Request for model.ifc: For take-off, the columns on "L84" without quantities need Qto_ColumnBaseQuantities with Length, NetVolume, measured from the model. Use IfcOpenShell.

First a look at what the model holds.

```python
import ifcopenshell
import ifcopenshell.util.element
import ifcopenshell.util.unit

model = ifcopenshell.open("model.ifc")
print(model.schema)
for unit_type in ("LENGTHUNIT", "AREAUNIT", "VOLUMEUNIT"):
    print(unit_type, ifcopenshell.util.unit.calculate_unit_scale(model, unit_type))
storey = next(s for s in model.by_type("IfcBuildingStorey") if s.Name == "L84")
columns = [e for e in ifcopenshell.util.element.get_decomposition(storey) if e.is_a("IfcColumn")]
for e in sorted(columns, key=lambda e: e.id()):
    print(e.id(), e.is_a(), e.Name, list(ifcopenshell.util.element.get_psets(e, qtos_only=True)), sep=" | ")
```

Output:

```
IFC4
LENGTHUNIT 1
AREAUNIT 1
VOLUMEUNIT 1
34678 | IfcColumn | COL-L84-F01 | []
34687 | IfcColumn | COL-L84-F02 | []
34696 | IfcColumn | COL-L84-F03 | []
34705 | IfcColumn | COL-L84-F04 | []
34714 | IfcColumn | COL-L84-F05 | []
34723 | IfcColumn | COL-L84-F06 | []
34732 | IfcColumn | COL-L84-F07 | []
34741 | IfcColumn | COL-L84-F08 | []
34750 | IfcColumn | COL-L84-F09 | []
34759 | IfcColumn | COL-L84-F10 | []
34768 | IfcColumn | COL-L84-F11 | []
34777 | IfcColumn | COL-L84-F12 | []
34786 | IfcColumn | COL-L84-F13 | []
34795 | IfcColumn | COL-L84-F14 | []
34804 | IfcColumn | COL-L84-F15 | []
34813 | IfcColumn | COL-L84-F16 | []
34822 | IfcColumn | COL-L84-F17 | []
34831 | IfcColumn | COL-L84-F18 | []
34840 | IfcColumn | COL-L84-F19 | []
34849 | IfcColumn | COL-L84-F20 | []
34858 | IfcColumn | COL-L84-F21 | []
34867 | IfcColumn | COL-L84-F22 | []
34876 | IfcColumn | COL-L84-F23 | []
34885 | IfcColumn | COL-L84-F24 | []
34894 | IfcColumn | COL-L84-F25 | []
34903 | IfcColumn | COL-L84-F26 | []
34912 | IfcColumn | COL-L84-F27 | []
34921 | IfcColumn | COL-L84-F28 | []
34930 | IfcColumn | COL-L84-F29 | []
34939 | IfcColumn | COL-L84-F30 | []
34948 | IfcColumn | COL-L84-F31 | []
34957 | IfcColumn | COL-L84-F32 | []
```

```python
import ifcopenshell
import ifcopenshell.api.pset
import ifcopenshell.geom
import ifcopenshell.util.element
import ifcopenshell.util.shape
import ifcopenshell.util.unit

model = ifcopenshell.open("model.ifc")
unit_scale = ifcopenshell.util.unit.calculate_unit_scale(model)
volume_scale = ifcopenshell.util.unit.calculate_unit_scale(model, "VOLUMEUNIT")
settings = ifcopenshell.geom.settings()

storey = next(s for s in model.by_type("IfcBuildingStorey") if s.Name == "L84")
columns = [e for e in ifcopenshell.util.element.get_decomposition(storey) if e.is_a("IfcColumn")]

for e in sorted(columns, key=lambda e: e.id()):
    if ifcopenshell.util.element.get_psets(e, qtos_only=True, should_inherit=False):
        continue
    # Geometry comes back in metres, in the element's own axes.
    shape = ifcopenshell.geom.create_shape(settings, e)
    values = {
        "Length": ifcopenshell.util.shape.get_z(shape.geometry) / unit_scale,
        "NetVolume": ifcopenshell.util.shape.get_volume(shape.geometry) / volume_scale,
    }
    qto = ifcopenshell.api.pset.add_qto(model, product=e, name="Qto_ColumnBaseQuantities")
    ifcopenshell.api.pset.edit_qto(model, qto=qto, properties=values)
    print(e.id(), {k: round(v, 3) for k, v in values.items()})

model.write("model_v2.ifc")
```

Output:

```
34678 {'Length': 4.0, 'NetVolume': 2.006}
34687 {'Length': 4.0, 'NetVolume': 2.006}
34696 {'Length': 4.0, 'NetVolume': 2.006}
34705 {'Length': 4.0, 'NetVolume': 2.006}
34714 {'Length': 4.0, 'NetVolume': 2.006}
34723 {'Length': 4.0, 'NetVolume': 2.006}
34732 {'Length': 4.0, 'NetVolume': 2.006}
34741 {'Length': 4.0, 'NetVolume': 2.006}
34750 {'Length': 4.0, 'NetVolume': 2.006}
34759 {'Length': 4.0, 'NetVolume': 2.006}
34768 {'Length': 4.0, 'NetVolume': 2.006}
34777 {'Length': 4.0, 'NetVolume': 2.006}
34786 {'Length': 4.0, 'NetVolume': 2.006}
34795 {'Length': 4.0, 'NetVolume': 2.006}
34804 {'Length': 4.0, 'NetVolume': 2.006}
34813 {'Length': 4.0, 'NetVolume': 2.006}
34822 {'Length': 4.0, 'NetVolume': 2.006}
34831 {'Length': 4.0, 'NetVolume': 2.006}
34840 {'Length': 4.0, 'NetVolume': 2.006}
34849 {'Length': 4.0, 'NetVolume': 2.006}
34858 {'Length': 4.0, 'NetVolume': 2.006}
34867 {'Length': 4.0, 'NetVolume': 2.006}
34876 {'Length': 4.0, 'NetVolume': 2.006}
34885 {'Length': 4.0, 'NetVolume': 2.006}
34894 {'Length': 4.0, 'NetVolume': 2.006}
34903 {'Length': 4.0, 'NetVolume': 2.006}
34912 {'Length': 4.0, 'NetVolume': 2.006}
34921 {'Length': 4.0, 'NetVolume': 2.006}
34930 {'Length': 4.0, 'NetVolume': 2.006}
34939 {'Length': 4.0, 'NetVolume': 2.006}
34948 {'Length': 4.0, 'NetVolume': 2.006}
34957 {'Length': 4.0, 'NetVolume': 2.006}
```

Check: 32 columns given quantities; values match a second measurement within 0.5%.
